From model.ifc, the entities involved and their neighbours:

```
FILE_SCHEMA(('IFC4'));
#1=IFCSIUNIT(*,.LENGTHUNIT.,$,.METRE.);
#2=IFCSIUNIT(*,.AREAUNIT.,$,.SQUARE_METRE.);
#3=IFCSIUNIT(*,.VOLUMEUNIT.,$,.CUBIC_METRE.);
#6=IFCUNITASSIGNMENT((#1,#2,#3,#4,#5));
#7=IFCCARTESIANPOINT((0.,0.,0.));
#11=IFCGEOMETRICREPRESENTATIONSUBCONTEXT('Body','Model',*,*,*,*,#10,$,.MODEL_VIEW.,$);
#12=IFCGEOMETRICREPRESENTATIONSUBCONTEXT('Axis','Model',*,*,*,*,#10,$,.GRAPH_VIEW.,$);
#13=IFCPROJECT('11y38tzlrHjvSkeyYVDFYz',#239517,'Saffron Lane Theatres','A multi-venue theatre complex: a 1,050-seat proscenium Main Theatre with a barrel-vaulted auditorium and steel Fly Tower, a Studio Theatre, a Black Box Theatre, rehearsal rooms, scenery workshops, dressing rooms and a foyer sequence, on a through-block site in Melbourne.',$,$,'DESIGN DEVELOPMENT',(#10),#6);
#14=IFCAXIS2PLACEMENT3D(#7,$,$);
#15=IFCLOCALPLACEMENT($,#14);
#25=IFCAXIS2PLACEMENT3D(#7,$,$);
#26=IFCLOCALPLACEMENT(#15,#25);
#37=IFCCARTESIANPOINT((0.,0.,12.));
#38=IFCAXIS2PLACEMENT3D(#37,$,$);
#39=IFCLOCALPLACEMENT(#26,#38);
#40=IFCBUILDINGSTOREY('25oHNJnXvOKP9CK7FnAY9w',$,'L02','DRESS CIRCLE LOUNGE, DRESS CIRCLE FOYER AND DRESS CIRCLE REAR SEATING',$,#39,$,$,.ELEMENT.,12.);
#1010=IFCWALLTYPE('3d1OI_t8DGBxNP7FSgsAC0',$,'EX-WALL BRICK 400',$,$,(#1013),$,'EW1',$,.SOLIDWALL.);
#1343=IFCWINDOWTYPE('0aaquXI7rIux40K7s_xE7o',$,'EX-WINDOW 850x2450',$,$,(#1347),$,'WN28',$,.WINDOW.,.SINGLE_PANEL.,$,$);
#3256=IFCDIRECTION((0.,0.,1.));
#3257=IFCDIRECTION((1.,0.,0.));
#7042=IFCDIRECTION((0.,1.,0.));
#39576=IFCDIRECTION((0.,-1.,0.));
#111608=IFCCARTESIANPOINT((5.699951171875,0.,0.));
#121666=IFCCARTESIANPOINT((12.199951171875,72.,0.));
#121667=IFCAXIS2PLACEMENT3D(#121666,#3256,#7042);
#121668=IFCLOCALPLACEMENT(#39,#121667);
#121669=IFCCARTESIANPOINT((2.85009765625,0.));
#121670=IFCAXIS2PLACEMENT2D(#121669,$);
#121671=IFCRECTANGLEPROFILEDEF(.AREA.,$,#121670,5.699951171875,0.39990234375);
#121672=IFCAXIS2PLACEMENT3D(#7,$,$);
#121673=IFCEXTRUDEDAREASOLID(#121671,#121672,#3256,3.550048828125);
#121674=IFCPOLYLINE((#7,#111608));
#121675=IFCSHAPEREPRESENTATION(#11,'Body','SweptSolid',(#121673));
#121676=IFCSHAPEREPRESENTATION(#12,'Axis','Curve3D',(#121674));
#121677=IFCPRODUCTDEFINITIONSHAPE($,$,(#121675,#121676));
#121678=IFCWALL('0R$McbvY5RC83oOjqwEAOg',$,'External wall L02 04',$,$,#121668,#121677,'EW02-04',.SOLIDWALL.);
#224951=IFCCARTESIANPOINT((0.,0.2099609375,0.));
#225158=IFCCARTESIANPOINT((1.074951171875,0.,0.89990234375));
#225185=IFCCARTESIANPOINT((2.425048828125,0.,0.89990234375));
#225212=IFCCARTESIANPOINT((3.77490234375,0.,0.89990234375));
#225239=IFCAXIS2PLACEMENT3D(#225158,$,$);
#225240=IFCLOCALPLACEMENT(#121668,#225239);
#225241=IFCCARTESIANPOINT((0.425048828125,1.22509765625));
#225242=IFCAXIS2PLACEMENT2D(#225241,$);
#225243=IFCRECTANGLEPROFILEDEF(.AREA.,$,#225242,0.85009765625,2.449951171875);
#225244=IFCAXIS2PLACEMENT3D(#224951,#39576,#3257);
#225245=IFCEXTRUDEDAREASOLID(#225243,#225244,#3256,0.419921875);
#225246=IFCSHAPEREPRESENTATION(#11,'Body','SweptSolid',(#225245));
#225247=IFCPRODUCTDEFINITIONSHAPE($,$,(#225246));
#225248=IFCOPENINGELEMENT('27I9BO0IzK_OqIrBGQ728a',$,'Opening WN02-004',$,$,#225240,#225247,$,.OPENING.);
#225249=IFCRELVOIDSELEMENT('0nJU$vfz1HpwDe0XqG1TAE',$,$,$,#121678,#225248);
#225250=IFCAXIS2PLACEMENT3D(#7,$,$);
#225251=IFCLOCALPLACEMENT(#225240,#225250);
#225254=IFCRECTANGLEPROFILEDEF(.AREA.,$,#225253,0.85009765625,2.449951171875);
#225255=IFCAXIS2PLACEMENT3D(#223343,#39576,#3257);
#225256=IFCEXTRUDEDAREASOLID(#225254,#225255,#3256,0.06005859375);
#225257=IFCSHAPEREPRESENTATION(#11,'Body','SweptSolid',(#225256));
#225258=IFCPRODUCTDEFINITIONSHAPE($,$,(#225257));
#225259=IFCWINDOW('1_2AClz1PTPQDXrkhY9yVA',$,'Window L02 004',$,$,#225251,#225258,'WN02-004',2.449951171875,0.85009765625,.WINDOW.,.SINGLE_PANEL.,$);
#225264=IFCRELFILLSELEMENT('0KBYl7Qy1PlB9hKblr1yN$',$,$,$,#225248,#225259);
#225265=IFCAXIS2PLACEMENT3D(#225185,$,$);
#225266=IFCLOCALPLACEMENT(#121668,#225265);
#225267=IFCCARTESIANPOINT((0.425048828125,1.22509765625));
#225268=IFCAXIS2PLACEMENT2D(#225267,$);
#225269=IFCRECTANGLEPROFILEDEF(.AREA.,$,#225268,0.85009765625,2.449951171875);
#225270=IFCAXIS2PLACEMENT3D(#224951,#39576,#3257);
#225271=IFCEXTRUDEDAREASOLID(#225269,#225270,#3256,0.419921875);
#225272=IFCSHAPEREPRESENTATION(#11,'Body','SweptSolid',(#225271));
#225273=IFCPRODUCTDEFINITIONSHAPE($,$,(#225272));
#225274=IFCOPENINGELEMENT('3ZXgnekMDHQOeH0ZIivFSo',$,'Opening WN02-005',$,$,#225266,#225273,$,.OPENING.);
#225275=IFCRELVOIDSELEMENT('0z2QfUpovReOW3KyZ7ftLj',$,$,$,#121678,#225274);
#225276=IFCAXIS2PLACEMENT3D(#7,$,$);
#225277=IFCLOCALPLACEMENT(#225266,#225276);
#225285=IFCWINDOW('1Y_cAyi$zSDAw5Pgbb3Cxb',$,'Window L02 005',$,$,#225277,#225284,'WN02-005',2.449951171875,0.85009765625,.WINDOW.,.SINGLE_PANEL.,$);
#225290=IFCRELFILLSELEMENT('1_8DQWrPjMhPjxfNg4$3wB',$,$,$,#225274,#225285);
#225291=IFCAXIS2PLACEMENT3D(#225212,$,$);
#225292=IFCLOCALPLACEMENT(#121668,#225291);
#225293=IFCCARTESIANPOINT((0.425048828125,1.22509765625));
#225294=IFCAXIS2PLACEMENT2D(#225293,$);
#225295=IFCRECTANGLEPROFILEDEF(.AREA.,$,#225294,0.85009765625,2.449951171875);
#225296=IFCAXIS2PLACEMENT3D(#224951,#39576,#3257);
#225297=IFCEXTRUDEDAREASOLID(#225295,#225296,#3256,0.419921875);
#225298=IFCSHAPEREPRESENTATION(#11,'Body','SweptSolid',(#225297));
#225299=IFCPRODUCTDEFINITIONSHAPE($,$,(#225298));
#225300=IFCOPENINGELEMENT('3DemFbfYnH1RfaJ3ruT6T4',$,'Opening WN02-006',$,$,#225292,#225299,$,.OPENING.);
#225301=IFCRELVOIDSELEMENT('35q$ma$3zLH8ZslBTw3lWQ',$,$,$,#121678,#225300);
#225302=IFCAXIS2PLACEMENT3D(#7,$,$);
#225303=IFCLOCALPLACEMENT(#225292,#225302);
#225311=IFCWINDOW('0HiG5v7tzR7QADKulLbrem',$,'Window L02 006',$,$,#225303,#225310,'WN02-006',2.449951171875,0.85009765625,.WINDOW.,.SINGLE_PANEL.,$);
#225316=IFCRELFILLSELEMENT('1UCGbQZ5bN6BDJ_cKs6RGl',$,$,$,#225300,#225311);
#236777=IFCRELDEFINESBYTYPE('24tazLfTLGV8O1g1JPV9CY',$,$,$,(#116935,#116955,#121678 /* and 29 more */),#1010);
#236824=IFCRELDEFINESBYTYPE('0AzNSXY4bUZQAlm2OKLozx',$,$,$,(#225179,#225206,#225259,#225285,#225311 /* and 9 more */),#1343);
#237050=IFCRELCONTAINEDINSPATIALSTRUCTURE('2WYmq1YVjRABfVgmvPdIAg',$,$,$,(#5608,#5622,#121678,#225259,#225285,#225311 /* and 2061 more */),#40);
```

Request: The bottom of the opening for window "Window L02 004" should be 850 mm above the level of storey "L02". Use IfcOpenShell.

```python
import numpy as np
import ifcopenshell
import ifcopenshell.api.geometry
import ifcopenshell.geom
import ifcopenshell.util.element
import ifcopenshell.util.placement
import ifcopenshell.util.shape
import ifcopenshell.util.unit

model = ifcopenshell.open("model.ifc")
unit_scale = ifcopenshell.util.unit.calculate_unit_scale(model)

window = model.by_guid("1_2AClz1PTPQDXrkhY9yVA")
opening = window.FillsVoids[0].RelatingOpeningElement
storey = ifcopenshell.util.element.get_container(window, ifc_class="IfcBuildingStorey")
level = ifcopenshell.util.placement.get_local_placement(storey.ObjectPlacement)[2, 3]

# The opening's origin need not be at the sill, so measure its lowest point.
shape = ifcopenshell.geom.create_shape(ifcopenshell.geom.settings(), opening)
bottom = ifcopenshell.util.shape.get_shape_bottom_elevation(shape, shape.geometry) / unit_scale
dz = level + 0.85 / unit_scale - bottom

shift = np.array([0.0, 0.0, dz])
# The window is placed relative to its opening, so it follows when the opening moves.
matrix = ifcopenshell.util.placement.get_local_placement(opening.ObjectPlacement)
matrix[:3, 3] += shift
ifcopenshell.api.geometry.edit_object_placement(
    model, product=opening, matrix=matrix, is_si=False, should_transform_children=True
)

print(f"moved by {dz * unit_scale:+.3f} m")

model.write("model_rev.ifc")
```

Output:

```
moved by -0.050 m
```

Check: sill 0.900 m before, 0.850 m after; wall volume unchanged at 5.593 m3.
